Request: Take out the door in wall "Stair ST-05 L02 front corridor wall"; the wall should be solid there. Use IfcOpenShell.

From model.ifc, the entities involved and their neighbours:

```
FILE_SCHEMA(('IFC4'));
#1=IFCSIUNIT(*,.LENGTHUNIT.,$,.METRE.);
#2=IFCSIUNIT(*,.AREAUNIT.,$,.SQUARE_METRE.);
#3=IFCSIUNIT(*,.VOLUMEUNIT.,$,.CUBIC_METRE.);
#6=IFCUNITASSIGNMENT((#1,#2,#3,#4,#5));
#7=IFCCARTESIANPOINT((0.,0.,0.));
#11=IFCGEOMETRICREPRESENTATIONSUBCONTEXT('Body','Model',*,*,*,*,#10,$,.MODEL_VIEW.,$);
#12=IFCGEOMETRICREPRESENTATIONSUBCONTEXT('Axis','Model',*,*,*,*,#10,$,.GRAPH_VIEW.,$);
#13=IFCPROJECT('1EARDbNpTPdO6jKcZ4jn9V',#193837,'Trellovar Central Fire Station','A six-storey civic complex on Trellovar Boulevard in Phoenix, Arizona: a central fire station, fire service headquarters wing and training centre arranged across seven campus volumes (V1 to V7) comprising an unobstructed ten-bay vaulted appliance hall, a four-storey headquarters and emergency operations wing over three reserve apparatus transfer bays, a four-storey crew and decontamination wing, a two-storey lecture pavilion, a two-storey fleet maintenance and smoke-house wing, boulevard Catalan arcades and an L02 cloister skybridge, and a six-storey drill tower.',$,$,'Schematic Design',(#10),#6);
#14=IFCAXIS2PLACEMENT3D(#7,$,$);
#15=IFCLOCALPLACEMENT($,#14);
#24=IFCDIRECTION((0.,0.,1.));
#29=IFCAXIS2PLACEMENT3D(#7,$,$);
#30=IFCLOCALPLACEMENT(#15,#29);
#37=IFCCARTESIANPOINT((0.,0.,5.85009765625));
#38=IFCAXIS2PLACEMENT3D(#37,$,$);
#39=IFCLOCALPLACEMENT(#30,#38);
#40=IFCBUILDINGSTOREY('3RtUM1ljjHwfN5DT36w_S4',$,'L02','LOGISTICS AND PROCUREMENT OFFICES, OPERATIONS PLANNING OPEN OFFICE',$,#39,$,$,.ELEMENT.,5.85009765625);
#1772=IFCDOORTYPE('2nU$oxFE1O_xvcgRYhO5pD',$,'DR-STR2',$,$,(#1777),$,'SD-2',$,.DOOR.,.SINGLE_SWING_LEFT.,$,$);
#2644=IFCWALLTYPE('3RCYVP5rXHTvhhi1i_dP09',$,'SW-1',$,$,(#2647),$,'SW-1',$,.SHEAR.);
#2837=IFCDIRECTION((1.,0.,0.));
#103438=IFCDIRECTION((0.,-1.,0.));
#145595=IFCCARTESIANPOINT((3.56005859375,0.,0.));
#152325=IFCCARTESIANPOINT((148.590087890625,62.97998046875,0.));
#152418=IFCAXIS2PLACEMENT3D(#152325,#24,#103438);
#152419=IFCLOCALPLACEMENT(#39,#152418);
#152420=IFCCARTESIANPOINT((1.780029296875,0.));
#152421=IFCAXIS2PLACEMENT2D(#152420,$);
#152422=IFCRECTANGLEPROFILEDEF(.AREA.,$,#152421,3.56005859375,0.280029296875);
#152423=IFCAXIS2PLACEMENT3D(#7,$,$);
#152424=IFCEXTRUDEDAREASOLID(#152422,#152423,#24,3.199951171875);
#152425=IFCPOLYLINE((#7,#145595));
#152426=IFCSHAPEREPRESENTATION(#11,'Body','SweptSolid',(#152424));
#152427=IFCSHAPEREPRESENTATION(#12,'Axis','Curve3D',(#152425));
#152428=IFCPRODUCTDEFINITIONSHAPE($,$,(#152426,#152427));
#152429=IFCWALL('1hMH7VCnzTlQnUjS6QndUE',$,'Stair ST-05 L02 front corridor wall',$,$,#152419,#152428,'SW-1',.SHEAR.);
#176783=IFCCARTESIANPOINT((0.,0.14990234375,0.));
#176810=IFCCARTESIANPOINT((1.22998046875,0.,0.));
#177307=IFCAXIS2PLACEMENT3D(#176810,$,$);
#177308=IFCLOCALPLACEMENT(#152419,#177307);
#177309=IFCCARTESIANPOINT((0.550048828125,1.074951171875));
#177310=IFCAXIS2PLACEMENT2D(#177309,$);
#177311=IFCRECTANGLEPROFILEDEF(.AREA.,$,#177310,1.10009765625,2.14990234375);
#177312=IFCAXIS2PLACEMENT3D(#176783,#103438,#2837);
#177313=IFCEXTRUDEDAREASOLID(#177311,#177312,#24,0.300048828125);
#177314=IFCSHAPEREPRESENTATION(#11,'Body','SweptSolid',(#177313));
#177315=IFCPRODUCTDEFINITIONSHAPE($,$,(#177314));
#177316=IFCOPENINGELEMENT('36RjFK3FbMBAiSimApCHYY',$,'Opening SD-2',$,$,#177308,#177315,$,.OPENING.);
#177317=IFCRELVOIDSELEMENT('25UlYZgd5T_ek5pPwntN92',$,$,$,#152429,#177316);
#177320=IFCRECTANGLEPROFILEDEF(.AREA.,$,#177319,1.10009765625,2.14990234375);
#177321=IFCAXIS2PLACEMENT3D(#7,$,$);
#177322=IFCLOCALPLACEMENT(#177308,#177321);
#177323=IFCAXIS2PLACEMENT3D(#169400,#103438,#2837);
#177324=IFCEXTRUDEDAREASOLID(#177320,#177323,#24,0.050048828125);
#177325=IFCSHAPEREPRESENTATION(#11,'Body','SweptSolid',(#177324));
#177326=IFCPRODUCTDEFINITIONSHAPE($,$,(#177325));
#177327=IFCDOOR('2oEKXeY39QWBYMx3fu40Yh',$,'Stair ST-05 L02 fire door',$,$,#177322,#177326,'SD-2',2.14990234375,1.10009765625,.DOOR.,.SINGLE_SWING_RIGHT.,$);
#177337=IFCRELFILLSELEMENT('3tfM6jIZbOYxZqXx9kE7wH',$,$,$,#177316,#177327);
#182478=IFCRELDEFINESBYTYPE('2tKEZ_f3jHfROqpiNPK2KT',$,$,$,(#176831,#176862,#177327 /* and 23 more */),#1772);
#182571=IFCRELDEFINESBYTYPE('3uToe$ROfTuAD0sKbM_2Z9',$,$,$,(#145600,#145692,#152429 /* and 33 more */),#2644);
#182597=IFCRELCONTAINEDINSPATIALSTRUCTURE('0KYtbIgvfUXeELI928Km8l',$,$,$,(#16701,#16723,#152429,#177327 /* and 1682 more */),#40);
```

```python
import ifcopenshell
import ifcopenshell.api.feature
import ifcopenshell.api.root
import ifcopenshell.geom
import ifcopenshell.util.shape

model = ifcopenshell.open("model.ifc")
settings = ifcopenshell.geom.settings()


def volume(element):
    """Net volume in cubic metres, openings subtracted."""
    shape = ifcopenshell.geom.create_shape(settings, element)
    return ifcopenshell.util.shape.get_volume(shape.geometry)


door = model.by_guid("2oEKXeY39QWBYMx3fu40Yh")
opening = door.FillsVoids[0].RelatingOpeningElement
wall = opening.VoidsElements[0].RelatingBuildingElement
before = volume(wall)

ifcopenshell.api.root.remove_product(model, product=door)
ifcopenshell.api.feature.remove_feature(model, feature=opening)

after = volume(wall)

print(f"wall volume {before:.3f} -> {after:.3f} m3")

model.write("model-out.ifc")
```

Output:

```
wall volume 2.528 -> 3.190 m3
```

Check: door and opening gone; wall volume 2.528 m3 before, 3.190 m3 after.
